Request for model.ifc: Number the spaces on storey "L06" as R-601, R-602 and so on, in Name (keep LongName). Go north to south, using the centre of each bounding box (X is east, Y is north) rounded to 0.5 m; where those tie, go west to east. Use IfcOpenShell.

First a look at what the model holds.

```python
import ifcopenshell
import ifcopenshell.util.element
import ifcopenshell.util.placement

model = ifcopenshell.open("model.ifc")
print(model.schema)
storey = next(s for s in model.by_type("IfcBuildingStorey") if s.Name == "L06")
spaces = [e for e in ifcopenshell.util.element.get_decomposition(storey) if e.is_a("IfcSpace")]
for e in sorted(spaces, key=lambda e: e.id()):
    origin = ifcopenshell.util.placement.get_local_placement(e.ObjectPlacement)[:3, 3]
    print(e.id(), e.Name, e.LongName, origin.round(2) + 0.0, sep=" | ")
```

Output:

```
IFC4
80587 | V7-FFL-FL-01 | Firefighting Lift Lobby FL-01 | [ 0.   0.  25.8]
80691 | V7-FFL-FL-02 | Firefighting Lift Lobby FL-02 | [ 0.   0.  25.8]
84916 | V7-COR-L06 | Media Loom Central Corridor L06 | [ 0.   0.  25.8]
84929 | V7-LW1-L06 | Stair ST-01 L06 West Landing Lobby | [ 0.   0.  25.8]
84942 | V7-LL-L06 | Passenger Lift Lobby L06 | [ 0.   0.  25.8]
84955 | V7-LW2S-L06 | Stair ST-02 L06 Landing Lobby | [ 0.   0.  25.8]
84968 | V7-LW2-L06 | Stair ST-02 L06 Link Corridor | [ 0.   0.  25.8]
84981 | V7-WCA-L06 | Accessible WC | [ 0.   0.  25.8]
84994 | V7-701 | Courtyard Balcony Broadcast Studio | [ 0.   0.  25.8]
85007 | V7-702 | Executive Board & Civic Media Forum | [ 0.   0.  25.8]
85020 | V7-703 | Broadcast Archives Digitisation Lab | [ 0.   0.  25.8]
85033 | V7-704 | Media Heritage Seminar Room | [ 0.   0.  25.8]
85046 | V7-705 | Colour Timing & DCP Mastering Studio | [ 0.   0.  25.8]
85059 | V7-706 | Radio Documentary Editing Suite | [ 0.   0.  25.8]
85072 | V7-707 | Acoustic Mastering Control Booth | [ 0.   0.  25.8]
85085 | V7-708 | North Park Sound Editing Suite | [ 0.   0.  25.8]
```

```python
import ifcopenshell
import ifcopenshell.geom
import ifcopenshell.util.element
import ifcopenshell.util.shape

model = ifcopenshell.open("model.ifc")
settings = ifcopenshell.geom.settings()
settings.set("use-world-coords", True)


def centre(element):
    shape = ifcopenshell.geom.create_shape(settings, element)
    return ifcopenshell.util.shape.get_bbox_centroid(shape.geometry)


storey = next(s for s in model.by_type("IfcBuildingStorey") if s.Name == "L06")
spaces = [e for e in ifcopenshell.util.element.get_decomposition(storey) if e.is_a("IfcSpace")]

# Insertion points can sit at a corner or the storey origin, so sort by the geometry (in metres).
centres = {e: centre(e) for e in spaces}
spaces.sort(key=lambda e: (-round(centres[e][1] / 0.5), centres[e][0]))

for i, e in enumerate(spaces, start=1):
    number = f"R-6{i:02d}"
    e.Name = number
    print(e.id(), number)

model.write("model-out.ifc")
```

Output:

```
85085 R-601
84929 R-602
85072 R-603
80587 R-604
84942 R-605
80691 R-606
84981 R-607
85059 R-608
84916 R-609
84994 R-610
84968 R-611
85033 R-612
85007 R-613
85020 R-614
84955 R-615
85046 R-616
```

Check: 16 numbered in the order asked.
